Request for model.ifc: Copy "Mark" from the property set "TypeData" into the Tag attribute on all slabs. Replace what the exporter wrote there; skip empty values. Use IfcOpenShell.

First a look at what the model holds.

```python
import ifcopenshell
import ifcopenshell.util.element

model = ifcopenshell.open("model.ifc")
print(model.schema)
slabs = model.by_type("IfcSlab")
print(len(slabs), "slabs")
for e in slabs[:8]:
    source = ifcopenshell.util.element.get_pset(e, "TypeData", "Mark")
    target = e.Tag
    print(e.id(), repr(source), repr(target), sep=" | ")
```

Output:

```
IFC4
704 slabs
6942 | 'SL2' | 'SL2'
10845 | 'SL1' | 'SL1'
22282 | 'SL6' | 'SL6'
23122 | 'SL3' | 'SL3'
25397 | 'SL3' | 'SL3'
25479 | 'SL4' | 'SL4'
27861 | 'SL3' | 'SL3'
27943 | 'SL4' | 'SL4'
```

```python
import ifcopenshell
import ifcopenshell.util.element

model = ifcopenshell.open("model.ifc")

count = 0
for e in model.by_type("IfcSlab"):
    value = ifcopenshell.util.element.get_pset(e, "TypeData", "Mark")
    current = e.Tag
    if not value or not value.strip() or current == value:
        continue
    e.Tag = value
    count += 1

print(count, "slabs updated")

model.write("model_updated.ifc")
```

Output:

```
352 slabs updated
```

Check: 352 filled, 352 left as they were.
